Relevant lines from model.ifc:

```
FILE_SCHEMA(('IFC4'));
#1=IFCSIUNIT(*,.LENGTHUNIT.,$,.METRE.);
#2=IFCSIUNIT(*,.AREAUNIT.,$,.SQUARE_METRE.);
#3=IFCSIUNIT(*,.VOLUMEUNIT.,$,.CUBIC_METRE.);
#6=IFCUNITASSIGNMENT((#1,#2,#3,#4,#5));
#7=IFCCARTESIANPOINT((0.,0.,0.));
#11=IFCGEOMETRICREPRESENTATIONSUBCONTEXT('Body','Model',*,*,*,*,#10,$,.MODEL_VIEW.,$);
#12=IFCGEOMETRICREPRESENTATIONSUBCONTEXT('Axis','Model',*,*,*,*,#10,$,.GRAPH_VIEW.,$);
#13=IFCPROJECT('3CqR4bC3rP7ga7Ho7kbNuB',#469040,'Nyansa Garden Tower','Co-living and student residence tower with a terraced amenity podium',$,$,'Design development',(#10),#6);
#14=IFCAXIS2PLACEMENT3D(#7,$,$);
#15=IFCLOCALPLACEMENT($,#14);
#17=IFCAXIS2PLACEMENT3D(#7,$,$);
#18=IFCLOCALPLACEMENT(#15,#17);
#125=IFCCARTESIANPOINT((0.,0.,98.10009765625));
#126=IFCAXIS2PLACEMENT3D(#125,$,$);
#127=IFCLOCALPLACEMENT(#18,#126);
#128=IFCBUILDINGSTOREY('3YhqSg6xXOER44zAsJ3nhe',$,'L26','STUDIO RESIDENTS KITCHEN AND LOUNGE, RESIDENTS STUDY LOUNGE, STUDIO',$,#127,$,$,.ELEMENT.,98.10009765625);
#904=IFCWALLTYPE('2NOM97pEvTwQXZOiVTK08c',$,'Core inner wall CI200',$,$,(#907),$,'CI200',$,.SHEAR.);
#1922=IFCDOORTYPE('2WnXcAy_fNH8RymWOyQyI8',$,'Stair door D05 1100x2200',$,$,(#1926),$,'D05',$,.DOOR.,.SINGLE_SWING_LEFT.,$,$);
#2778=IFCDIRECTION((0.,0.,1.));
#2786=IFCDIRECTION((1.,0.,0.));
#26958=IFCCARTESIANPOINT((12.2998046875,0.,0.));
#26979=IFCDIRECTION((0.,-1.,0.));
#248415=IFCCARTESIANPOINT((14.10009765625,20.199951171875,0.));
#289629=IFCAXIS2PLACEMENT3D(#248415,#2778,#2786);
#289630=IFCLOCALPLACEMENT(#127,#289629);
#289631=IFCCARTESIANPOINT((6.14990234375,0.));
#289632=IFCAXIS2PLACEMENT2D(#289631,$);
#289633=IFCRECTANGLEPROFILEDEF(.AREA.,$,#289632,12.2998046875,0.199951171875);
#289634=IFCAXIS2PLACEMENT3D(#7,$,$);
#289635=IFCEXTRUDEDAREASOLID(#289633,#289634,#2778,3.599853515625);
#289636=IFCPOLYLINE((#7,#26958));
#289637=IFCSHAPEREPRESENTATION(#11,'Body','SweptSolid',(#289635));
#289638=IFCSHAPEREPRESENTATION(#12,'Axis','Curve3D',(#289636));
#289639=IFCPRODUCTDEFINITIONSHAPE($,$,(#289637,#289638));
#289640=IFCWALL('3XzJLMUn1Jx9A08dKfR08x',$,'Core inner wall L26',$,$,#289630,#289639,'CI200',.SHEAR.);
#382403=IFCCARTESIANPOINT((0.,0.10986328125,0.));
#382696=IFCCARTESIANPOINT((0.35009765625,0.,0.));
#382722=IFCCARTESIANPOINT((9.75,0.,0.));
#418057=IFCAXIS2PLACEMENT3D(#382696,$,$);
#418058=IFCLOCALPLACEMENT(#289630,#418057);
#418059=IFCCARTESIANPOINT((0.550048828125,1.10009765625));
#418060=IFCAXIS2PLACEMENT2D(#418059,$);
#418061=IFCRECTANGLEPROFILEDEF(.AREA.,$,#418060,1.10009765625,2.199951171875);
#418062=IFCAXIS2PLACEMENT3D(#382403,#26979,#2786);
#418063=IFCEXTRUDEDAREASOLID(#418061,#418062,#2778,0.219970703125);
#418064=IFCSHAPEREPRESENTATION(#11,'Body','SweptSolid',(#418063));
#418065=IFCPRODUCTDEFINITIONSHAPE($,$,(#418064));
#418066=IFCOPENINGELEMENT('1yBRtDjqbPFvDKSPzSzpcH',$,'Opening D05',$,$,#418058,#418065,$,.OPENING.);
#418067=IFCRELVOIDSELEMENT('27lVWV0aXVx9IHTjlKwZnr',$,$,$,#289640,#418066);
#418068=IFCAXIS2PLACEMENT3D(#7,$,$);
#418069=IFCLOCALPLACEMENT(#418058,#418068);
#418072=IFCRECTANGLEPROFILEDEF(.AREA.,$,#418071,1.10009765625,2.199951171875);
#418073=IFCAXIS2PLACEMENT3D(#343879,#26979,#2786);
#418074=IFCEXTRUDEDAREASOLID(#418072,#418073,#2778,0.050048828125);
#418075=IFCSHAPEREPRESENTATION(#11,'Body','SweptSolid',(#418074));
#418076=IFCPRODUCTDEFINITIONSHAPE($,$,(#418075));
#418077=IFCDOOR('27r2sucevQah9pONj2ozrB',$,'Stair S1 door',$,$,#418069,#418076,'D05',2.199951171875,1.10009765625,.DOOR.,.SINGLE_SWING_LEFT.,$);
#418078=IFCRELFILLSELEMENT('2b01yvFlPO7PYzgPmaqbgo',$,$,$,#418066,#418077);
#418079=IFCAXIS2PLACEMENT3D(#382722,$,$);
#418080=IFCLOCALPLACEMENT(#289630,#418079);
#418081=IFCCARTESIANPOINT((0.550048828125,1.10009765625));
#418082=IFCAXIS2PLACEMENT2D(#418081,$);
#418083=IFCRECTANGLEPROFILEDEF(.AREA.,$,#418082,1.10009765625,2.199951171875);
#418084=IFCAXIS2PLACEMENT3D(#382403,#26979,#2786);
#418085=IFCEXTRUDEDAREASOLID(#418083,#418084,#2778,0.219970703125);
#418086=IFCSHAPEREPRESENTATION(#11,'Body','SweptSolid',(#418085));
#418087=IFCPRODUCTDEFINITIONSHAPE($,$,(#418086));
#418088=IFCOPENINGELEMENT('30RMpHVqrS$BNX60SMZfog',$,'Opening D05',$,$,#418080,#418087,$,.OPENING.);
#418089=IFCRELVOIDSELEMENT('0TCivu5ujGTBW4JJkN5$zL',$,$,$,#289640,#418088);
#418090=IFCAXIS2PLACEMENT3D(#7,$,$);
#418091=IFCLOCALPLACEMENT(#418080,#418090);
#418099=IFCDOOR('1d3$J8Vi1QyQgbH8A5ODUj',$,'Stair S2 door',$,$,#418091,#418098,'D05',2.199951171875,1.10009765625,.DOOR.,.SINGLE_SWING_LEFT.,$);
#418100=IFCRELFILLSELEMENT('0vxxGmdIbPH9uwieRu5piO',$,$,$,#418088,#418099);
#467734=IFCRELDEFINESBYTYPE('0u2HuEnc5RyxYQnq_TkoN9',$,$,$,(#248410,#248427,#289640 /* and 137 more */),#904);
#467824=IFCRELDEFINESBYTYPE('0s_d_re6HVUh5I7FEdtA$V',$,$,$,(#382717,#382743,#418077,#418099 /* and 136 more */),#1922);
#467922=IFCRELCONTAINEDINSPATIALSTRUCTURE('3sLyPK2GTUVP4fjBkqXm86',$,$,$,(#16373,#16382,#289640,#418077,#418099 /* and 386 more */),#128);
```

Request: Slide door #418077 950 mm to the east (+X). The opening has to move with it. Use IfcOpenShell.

```python
import ifcopenshell
import ifcopenshell.api.geometry
import ifcopenshell.util.placement

model = ifcopenshell.open("model.ifc")

door = model.by_guid("27r2sucevQah9pONj2ozrB")
opening = door.FillsVoids[0].RelatingOpeningElement
wall = opening.VoidsElements[0].RelatingBuildingElement

wall_matrix = ifcopenshell.util.placement.get_local_placement(wall.ObjectPlacement)
shift = wall_matrix[:3, 0] * 0.95
before = ifcopenshell.util.placement.get_local_placement(door.ObjectPlacement)[:3, 3].copy()

# The door is placed relative to its opening, so it follows when the opening moves.
matrix = ifcopenshell.util.placement.get_local_placement(opening.ObjectPlacement)
matrix[:3, 3] += shift
ifcopenshell.api.geometry.edit_object_placement(
    model, product=opening, matrix=matrix, is_si=False, should_transform_children=True
)

after = ifcopenshell.util.placement.get_local_placement(door.ObjectPlacement)[:3, 3]
print("door moved by", (after - before).round(3) + 0.0)

model.write("model_v2.ifc")
```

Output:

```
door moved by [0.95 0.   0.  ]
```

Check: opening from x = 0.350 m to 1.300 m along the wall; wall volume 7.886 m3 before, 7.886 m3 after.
